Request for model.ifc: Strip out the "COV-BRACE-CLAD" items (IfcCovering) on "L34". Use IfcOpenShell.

First a look at what the model holds.

```python
import ifcopenshell
import ifcopenshell.util.element

model = ifcopenshell.open("model.ifc")
print(model.schema)
storey = next(s for s in model.by_type("IfcBuildingStorey") if s.Name == "L34")
coverings = [e for e in ifcopenshell.util.element.get_decomposition(storey) if e.is_a("IfcCovering")]
seen = {}
for e in coverings:
    element_type = ifcopenshell.util.element.get_type(e)
    name = element_type.Name if element_type not in (None, e) else None
    seen[name] = seen.get(name, 0) + 1
for name, count in sorted(seen.items(), key=str):
    print(count, "x", name)
```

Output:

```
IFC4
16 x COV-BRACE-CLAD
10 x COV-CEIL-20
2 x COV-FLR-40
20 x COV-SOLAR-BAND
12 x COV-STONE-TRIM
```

```python
import ifcopenshell
import ifcopenshell.api.root
import ifcopenshell.util.element

model = ifcopenshell.open("model.ifc")

storey = next(s for s in model.by_type("IfcBuildingStorey") if s.Name == "L34")
coverings = [e for e in ifcopenshell.util.element.get_decomposition(storey) if e.is_a("IfcCovering")]
targets = [e for e in coverings if (t := ifcopenshell.util.element.get_type(e)) not in (None, e) and t.Name == "COV-BRACE-CLAD"]

for e in targets:
    ifcopenshell.api.root.remove_product(model, product=e)
print(len(targets), "removed")

model.write("model_updated.ifc")
```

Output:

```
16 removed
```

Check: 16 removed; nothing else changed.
